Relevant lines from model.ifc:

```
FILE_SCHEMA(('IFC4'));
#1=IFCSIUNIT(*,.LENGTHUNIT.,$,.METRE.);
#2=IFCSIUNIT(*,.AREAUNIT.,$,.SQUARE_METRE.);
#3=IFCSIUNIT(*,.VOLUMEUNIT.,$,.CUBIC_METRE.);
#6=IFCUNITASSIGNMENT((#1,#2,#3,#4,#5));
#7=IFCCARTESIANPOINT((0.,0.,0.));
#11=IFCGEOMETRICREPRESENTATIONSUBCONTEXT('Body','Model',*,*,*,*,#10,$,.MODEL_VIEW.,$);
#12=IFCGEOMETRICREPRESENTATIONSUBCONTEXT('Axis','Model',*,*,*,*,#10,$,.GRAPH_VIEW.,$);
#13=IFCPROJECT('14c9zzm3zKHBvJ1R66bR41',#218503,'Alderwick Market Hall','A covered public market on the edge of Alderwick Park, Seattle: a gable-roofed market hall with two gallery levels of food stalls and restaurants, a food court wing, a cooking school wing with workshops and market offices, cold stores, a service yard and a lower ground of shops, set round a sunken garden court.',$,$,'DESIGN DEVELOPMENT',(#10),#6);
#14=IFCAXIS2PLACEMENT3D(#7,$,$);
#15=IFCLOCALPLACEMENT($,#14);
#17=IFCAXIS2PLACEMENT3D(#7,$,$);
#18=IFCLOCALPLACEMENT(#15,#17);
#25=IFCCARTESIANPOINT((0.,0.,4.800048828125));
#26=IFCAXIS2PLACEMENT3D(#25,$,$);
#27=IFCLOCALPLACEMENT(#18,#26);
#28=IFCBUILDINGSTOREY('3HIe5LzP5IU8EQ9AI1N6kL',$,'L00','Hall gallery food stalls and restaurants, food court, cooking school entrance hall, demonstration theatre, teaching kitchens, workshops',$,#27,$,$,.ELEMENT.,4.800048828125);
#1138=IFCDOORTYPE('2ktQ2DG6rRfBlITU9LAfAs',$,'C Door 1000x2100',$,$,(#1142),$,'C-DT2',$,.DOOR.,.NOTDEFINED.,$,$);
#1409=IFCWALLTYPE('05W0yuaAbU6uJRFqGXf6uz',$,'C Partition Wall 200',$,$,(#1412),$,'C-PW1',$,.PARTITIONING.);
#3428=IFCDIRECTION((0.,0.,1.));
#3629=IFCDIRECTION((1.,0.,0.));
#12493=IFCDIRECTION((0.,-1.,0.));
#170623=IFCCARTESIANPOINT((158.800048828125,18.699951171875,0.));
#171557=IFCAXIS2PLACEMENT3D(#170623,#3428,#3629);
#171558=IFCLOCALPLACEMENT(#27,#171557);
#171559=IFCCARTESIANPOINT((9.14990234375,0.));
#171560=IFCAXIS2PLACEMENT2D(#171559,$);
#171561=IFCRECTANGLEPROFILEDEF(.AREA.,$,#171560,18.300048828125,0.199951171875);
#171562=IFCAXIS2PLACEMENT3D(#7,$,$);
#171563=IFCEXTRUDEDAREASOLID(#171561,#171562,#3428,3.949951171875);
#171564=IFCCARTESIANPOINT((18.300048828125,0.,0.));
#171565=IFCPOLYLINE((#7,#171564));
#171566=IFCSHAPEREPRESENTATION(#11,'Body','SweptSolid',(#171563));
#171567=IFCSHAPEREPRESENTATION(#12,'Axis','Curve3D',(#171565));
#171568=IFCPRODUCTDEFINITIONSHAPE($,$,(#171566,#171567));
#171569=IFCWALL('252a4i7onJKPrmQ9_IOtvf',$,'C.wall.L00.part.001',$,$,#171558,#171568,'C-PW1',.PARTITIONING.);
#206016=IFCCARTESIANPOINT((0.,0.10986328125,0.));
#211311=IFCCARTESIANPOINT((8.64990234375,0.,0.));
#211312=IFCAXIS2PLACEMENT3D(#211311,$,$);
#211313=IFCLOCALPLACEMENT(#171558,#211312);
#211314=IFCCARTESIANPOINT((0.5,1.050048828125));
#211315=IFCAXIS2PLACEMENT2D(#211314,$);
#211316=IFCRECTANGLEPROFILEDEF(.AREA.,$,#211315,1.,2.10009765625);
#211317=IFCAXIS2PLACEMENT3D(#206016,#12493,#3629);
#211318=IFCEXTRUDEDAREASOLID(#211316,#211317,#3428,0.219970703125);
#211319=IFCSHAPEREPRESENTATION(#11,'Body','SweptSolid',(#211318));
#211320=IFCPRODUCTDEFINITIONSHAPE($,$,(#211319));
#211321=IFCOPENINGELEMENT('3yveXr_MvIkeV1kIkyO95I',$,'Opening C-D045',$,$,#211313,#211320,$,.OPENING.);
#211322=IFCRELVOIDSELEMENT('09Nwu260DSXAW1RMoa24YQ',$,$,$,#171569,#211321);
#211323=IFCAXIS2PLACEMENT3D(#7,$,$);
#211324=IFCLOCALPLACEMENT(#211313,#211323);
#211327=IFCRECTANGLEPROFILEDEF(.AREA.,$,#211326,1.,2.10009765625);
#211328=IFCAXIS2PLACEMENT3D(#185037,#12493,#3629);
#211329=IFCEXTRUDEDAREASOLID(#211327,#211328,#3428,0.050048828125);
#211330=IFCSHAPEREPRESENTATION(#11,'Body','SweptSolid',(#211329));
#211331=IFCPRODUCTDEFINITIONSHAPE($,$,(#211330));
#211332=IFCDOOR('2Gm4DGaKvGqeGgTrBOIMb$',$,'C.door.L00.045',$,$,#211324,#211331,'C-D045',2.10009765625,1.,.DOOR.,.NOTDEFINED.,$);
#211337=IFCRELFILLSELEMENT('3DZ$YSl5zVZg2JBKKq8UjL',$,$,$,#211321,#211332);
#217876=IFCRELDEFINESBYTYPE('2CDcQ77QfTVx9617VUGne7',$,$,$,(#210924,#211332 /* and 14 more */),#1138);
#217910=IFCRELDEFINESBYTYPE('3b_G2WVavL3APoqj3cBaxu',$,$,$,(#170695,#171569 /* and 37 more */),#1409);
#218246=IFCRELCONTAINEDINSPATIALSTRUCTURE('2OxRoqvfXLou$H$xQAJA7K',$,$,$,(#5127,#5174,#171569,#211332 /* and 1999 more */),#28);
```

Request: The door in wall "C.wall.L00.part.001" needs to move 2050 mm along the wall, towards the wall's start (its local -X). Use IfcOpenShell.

```python
import ifcopenshell
import ifcopenshell.api.geometry
import ifcopenshell.util.placement

model = ifcopenshell.open("model.ifc")

door = model.by_guid("2Gm4DGaKvGqeGgTrBOIMb$")
opening = door.FillsVoids[0].RelatingOpeningElement
wall = opening.VoidsElements[0].RelatingBuildingElement

wall_matrix = ifcopenshell.util.placement.get_local_placement(wall.ObjectPlacement)
shift = wall_matrix[:3, 0] * -2.05
before = ifcopenshell.util.placement.get_local_placement(door.ObjectPlacement)[:3, 3].copy()

# The door is placed relative to its opening, so it follows when the opening moves.
matrix = ifcopenshell.util.placement.get_local_placement(opening.ObjectPlacement)
matrix[:3, 3] += shift
ifcopenshell.api.geometry.edit_object_placement(
    model, product=opening, matrix=matrix, is_si=False, should_transform_children=True
)

after = ifcopenshell.util.placement.get_local_placement(door.ObjectPlacement)[:3, 3]
print("door moved by", (after - before).round(3) + 0.0)

model.write("model-out.ifc")
```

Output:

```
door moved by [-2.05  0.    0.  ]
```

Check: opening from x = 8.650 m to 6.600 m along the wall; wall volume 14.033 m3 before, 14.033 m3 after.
